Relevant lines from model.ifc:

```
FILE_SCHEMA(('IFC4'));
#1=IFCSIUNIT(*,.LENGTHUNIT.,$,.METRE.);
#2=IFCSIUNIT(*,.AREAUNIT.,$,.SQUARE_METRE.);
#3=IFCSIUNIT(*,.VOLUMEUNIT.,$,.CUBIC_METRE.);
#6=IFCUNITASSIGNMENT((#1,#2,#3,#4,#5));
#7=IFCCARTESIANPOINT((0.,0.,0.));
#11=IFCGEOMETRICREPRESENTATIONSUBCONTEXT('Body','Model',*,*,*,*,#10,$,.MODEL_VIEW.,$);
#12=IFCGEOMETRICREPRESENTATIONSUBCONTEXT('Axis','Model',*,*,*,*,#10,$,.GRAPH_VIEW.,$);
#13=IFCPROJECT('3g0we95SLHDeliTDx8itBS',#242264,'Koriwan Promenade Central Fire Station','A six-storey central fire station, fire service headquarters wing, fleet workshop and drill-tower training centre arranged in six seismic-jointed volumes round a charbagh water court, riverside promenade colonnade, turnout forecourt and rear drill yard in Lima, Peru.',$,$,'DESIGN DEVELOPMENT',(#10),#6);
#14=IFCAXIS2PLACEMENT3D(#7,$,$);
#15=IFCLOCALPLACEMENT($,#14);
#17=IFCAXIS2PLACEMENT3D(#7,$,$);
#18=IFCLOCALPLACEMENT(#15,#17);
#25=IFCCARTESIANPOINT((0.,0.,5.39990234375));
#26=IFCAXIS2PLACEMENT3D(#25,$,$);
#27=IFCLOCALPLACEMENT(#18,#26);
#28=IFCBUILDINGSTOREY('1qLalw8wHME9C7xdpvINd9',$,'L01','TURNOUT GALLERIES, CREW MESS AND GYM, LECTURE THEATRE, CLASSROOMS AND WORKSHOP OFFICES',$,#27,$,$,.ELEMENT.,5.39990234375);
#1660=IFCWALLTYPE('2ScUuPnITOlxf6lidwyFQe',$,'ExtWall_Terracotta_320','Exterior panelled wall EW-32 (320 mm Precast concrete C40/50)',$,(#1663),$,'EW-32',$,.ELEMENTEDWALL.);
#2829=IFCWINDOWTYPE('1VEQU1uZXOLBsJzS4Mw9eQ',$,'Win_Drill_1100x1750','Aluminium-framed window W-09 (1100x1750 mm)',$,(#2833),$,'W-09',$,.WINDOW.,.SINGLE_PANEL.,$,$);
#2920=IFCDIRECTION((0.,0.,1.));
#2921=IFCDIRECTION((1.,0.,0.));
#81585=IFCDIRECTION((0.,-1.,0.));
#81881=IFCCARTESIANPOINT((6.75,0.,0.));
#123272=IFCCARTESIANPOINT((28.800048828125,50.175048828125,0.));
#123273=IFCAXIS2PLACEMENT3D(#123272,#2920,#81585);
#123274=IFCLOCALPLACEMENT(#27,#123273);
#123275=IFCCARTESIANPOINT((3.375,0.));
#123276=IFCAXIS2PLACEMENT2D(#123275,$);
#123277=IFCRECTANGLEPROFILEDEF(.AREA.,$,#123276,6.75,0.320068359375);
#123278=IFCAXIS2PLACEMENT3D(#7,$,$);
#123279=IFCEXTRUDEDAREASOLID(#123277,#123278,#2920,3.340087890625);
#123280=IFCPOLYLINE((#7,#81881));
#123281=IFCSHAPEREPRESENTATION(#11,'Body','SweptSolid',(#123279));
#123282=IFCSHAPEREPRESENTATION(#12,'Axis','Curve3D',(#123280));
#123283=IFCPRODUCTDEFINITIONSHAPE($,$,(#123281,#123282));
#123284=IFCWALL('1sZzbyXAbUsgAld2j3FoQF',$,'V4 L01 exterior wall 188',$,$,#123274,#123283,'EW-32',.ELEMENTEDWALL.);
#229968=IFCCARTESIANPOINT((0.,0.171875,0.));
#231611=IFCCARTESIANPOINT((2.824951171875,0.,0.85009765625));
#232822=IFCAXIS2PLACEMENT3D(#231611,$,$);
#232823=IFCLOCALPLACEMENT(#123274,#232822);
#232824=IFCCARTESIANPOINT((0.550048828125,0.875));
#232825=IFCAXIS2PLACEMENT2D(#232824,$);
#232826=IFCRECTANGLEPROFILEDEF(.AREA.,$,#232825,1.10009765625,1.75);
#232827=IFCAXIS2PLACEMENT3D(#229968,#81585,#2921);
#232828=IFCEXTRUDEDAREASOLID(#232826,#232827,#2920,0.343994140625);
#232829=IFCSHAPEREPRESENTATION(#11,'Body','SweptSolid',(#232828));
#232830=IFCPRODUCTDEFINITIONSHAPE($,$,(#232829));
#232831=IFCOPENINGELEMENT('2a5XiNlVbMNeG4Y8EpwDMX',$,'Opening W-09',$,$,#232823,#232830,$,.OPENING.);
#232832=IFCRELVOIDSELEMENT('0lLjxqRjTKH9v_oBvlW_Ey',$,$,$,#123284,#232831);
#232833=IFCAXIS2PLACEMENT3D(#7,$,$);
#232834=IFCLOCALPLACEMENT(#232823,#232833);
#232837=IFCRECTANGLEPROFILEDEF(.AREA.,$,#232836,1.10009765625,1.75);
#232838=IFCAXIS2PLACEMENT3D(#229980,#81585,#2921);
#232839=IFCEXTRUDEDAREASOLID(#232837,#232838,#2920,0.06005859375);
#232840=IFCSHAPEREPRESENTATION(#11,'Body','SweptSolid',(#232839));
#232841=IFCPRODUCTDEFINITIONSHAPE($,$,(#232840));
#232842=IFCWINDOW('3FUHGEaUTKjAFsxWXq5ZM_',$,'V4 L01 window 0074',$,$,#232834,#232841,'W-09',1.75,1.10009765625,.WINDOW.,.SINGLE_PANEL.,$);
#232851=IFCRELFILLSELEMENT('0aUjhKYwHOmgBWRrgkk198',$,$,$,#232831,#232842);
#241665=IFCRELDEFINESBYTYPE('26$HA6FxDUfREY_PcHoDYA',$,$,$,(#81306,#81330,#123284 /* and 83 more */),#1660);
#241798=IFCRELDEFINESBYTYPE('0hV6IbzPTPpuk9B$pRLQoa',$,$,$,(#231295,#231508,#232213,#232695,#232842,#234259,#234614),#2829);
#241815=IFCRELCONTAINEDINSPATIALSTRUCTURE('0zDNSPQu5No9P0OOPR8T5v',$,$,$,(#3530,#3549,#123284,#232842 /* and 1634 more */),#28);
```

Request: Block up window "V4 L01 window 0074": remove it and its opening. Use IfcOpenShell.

```python
import ifcopenshell
import ifcopenshell.api.feature
import ifcopenshell.api.root
import ifcopenshell.geom
import ifcopenshell.util.shape

model = ifcopenshell.open("model.ifc")
settings = ifcopenshell.geom.settings()


def volume(element):
    """Net volume in cubic metres, openings subtracted."""
    shape = ifcopenshell.geom.create_shape(settings, element)
    return ifcopenshell.util.shape.get_volume(shape.geometry)


window = model.by_guid("3FUHGEaUTKjAFsxWXq5ZM_")
opening = window.FillsVoids[0].RelatingOpeningElement
wall = opening.VoidsElements[0].RelatingBuildingElement
before = volume(wall)

ifcopenshell.api.root.remove_product(model, product=window)
ifcopenshell.api.feature.remove_feature(model, feature=opening)

after = volume(wall)

print(f"wall volume {before:.3f} -> {after:.3f} m3")

model.write("model_rev.ifc")
```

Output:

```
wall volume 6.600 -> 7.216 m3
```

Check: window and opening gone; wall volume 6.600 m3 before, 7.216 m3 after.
